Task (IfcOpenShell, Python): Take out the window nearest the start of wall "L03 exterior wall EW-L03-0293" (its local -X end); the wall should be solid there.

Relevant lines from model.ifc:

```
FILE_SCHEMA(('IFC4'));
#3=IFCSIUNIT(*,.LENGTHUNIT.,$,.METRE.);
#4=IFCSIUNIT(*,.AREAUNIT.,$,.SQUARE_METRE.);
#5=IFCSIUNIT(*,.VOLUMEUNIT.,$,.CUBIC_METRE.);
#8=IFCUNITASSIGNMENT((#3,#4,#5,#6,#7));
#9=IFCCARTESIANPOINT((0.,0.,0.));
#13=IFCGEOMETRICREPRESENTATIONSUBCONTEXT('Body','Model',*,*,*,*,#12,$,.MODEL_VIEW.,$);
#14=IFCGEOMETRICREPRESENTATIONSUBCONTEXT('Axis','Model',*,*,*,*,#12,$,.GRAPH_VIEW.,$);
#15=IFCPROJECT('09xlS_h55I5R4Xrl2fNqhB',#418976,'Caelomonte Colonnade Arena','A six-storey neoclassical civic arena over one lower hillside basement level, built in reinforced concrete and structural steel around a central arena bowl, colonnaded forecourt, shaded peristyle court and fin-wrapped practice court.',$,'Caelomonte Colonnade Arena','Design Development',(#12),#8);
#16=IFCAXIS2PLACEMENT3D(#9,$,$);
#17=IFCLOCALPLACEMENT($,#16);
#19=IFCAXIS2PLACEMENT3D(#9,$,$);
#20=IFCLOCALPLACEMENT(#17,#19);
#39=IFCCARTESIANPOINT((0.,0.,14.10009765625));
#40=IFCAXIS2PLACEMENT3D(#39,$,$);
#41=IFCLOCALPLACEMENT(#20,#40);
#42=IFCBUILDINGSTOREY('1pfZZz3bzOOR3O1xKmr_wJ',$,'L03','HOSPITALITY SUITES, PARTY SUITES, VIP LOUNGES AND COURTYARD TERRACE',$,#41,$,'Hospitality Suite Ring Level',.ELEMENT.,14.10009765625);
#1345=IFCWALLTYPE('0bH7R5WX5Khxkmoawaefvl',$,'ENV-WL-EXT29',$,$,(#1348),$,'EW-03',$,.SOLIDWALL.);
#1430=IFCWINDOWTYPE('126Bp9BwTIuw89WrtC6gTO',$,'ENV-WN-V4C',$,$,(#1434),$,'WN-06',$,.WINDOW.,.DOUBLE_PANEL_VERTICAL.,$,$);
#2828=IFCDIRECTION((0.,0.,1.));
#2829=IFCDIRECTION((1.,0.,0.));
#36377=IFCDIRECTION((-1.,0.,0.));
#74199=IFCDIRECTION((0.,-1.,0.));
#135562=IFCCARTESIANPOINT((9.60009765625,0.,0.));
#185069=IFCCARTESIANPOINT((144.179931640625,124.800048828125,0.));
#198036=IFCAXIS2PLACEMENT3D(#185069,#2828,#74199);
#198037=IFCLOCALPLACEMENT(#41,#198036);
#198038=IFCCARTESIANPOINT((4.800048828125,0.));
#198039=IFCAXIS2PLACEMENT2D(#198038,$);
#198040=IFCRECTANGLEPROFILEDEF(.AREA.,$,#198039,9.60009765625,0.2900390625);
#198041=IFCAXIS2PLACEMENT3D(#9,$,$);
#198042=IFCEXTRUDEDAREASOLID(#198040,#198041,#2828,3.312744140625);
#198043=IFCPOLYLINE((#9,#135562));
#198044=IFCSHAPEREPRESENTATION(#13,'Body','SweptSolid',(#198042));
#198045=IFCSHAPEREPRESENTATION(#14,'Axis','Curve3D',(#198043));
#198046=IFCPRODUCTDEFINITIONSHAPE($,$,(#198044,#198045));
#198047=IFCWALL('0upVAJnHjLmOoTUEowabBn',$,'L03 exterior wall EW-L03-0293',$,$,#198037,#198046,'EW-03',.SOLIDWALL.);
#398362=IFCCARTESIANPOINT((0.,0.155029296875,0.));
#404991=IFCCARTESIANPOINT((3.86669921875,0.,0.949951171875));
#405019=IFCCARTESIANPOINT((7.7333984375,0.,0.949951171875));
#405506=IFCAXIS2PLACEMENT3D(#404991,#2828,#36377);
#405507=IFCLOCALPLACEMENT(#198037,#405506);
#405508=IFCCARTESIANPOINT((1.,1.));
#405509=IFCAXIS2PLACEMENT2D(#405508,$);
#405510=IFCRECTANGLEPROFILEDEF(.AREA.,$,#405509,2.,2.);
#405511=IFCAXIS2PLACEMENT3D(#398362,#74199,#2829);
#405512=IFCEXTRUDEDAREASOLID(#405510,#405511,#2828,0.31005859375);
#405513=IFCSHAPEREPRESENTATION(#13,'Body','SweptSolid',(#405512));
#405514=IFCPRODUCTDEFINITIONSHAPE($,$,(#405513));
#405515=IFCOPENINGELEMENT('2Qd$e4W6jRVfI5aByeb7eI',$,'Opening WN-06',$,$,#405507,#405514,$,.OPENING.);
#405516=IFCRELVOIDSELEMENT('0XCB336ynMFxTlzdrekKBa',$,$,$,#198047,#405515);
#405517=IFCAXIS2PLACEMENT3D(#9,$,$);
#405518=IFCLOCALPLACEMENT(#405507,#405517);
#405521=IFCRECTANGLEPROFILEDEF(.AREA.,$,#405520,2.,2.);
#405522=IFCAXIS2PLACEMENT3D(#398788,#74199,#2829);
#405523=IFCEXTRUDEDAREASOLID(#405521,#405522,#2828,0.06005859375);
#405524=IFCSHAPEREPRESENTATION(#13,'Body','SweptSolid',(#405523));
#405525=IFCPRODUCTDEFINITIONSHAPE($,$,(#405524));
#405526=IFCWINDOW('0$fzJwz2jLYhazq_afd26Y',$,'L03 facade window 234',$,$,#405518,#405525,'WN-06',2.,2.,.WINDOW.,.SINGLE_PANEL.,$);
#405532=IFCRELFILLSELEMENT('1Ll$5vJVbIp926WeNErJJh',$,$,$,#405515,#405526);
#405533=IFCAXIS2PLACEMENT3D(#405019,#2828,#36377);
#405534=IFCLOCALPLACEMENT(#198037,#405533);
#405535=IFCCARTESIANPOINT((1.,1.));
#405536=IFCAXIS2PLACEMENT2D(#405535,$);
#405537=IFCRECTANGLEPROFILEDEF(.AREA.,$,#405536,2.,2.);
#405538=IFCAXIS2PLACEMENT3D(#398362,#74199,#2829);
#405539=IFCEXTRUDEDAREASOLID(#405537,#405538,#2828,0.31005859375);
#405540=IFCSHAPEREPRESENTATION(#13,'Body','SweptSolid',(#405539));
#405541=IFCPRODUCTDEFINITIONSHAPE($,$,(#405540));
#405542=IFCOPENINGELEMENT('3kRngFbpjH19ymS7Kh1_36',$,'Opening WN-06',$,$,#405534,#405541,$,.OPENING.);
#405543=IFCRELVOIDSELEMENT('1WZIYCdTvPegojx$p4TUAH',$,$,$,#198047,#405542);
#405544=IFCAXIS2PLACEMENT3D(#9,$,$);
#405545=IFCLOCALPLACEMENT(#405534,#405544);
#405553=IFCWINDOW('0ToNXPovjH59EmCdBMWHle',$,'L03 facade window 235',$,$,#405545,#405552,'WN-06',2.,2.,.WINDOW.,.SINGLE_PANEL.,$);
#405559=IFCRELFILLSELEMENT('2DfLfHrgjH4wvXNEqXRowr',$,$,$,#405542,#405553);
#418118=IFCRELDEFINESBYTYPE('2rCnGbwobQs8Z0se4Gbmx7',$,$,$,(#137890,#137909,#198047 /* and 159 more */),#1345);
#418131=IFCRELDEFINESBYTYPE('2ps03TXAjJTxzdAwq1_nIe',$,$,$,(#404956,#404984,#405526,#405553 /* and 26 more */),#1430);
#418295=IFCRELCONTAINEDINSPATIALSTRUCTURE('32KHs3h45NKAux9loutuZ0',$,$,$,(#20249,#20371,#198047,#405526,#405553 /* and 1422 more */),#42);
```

```python
import ifcopenshell
import ifcopenshell.api.feature
import ifcopenshell.api.root
import ifcopenshell.geom
import ifcopenshell.util.shape

model = ifcopenshell.open("model.ifc")
settings = ifcopenshell.geom.settings()


def volume(element):
    """Net volume in cubic metres, openings subtracted."""
    shape = ifcopenshell.geom.create_shape(settings, element)
    return ifcopenshell.util.shape.get_volume(shape.geometry)


window = model.by_guid("0$fzJwz2jLYhazq_afd26Y")
opening = window.FillsVoids[0].RelatingOpeningElement
wall = opening.VoidsElements[0].RelatingBuildingElement
before = volume(wall)

ifcopenshell.api.root.remove_product(model, product=window)
ifcopenshell.api.feature.remove_feature(model, feature=opening)

after = volume(wall)

print(f"wall volume {before:.3f} -> {after:.3f} m3")

model.write("model_v2.ifc")
```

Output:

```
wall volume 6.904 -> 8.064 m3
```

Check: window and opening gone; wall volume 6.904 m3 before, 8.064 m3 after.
